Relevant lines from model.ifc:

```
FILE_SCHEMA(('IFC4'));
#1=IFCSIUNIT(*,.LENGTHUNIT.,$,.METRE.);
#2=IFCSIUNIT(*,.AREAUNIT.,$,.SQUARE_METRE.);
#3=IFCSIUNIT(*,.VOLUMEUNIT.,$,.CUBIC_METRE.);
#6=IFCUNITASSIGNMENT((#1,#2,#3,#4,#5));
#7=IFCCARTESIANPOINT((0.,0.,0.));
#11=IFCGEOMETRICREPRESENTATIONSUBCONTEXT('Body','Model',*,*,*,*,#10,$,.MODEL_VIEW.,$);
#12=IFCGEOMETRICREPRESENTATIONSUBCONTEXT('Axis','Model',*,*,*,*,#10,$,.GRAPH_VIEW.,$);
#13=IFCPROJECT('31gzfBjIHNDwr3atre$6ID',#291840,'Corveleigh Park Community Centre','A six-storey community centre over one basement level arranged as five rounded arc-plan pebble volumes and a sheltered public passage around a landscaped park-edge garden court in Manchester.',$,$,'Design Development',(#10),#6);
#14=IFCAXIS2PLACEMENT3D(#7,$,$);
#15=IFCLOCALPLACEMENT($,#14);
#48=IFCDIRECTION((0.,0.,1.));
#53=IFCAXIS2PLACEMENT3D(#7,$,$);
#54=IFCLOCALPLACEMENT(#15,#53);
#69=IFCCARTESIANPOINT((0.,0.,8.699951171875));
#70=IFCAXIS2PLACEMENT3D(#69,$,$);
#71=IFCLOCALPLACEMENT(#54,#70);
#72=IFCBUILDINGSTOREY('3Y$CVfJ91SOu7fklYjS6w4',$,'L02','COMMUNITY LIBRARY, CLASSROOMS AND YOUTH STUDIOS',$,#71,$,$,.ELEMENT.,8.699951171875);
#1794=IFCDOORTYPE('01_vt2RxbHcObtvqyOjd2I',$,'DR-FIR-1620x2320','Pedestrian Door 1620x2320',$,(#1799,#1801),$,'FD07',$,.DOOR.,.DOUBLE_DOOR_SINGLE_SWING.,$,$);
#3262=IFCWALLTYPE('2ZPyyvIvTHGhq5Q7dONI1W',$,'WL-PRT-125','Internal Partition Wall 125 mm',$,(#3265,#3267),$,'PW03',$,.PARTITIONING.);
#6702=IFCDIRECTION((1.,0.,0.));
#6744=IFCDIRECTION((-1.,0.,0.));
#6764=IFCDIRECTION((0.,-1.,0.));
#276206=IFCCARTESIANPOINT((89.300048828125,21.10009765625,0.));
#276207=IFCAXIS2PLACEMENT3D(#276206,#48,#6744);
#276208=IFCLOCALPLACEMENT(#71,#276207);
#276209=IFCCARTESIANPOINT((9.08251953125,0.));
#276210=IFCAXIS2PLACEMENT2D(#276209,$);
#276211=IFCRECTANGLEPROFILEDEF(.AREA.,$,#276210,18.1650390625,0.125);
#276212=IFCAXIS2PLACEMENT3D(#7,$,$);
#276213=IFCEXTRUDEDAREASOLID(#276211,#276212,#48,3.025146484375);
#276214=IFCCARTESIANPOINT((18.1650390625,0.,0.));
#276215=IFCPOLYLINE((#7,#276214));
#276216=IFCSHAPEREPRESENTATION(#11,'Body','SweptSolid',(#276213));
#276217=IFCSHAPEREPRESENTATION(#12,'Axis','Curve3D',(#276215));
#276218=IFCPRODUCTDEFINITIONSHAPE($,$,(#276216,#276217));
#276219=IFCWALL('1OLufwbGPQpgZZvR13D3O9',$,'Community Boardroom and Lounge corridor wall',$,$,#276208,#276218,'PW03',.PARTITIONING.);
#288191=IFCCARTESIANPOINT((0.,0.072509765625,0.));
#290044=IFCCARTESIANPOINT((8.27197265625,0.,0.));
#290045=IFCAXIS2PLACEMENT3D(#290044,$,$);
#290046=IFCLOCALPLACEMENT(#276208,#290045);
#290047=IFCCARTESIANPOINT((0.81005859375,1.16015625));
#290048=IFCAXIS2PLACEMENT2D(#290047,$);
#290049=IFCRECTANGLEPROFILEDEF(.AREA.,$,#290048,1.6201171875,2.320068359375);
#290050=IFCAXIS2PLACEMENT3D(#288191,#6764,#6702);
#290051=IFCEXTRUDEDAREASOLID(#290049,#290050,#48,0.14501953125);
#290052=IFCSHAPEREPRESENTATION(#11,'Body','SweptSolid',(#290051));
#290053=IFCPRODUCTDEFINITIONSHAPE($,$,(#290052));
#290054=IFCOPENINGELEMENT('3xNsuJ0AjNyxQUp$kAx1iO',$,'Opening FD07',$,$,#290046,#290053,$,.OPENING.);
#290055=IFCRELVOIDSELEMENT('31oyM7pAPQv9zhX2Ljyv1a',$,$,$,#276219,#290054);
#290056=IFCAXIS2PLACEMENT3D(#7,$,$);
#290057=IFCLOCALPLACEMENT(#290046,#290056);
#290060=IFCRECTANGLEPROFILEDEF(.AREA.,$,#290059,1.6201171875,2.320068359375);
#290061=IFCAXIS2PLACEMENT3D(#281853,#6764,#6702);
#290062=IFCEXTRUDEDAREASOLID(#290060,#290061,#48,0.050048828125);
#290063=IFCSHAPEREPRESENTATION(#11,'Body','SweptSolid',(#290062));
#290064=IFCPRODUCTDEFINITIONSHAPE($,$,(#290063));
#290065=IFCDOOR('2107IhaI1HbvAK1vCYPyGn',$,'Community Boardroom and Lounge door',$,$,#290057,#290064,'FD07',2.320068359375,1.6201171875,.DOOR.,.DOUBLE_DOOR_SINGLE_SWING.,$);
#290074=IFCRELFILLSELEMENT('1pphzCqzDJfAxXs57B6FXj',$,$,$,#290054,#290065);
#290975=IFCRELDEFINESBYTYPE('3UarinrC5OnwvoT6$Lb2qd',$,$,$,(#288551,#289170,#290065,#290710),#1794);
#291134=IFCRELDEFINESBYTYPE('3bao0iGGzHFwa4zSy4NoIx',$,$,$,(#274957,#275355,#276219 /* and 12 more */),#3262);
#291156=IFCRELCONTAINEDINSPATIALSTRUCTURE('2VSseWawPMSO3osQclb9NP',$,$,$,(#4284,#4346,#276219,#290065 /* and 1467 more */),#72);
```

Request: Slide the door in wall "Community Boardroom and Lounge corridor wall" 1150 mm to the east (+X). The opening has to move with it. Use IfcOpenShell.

```python
import ifcopenshell
import ifcopenshell.api.geometry
import ifcopenshell.util.placement
import ifcopenshell.util.unit

model = ifcopenshell.open("model.ifc")
unit_scale = ifcopenshell.util.unit.calculate_unit_scale(model)

door = model.by_guid("2107IhaI1HbvAK1vCYPyGn")
opening = door.FillsVoids[0].RelatingOpeningElement
wall = opening.VoidsElements[0].RelatingBuildingElement

wall_matrix = ifcopenshell.util.placement.get_local_placement(wall.ObjectPlacement)
shift = wall_matrix[:3, 0] * -1.15 / unit_scale
before = ifcopenshell.util.placement.get_local_placement(door.ObjectPlacement)[:3, 3].copy()

# The door is placed relative to its opening, so it follows when the opening moves.
matrix = ifcopenshell.util.placement.get_local_placement(opening.ObjectPlacement)
matrix[:3, 3] += shift
ifcopenshell.api.geometry.edit_object_placement(
    model, product=opening, matrix=matrix, is_si=False, should_transform_children=True
)

after = ifcopenshell.util.placement.get_local_placement(door.ObjectPlacement)[:3, 3]
print("door moved by", (after - before).round(3) + 0.0)

model.write("model_rev.ifc")
```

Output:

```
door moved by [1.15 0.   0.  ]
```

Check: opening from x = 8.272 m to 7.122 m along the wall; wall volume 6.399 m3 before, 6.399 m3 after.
